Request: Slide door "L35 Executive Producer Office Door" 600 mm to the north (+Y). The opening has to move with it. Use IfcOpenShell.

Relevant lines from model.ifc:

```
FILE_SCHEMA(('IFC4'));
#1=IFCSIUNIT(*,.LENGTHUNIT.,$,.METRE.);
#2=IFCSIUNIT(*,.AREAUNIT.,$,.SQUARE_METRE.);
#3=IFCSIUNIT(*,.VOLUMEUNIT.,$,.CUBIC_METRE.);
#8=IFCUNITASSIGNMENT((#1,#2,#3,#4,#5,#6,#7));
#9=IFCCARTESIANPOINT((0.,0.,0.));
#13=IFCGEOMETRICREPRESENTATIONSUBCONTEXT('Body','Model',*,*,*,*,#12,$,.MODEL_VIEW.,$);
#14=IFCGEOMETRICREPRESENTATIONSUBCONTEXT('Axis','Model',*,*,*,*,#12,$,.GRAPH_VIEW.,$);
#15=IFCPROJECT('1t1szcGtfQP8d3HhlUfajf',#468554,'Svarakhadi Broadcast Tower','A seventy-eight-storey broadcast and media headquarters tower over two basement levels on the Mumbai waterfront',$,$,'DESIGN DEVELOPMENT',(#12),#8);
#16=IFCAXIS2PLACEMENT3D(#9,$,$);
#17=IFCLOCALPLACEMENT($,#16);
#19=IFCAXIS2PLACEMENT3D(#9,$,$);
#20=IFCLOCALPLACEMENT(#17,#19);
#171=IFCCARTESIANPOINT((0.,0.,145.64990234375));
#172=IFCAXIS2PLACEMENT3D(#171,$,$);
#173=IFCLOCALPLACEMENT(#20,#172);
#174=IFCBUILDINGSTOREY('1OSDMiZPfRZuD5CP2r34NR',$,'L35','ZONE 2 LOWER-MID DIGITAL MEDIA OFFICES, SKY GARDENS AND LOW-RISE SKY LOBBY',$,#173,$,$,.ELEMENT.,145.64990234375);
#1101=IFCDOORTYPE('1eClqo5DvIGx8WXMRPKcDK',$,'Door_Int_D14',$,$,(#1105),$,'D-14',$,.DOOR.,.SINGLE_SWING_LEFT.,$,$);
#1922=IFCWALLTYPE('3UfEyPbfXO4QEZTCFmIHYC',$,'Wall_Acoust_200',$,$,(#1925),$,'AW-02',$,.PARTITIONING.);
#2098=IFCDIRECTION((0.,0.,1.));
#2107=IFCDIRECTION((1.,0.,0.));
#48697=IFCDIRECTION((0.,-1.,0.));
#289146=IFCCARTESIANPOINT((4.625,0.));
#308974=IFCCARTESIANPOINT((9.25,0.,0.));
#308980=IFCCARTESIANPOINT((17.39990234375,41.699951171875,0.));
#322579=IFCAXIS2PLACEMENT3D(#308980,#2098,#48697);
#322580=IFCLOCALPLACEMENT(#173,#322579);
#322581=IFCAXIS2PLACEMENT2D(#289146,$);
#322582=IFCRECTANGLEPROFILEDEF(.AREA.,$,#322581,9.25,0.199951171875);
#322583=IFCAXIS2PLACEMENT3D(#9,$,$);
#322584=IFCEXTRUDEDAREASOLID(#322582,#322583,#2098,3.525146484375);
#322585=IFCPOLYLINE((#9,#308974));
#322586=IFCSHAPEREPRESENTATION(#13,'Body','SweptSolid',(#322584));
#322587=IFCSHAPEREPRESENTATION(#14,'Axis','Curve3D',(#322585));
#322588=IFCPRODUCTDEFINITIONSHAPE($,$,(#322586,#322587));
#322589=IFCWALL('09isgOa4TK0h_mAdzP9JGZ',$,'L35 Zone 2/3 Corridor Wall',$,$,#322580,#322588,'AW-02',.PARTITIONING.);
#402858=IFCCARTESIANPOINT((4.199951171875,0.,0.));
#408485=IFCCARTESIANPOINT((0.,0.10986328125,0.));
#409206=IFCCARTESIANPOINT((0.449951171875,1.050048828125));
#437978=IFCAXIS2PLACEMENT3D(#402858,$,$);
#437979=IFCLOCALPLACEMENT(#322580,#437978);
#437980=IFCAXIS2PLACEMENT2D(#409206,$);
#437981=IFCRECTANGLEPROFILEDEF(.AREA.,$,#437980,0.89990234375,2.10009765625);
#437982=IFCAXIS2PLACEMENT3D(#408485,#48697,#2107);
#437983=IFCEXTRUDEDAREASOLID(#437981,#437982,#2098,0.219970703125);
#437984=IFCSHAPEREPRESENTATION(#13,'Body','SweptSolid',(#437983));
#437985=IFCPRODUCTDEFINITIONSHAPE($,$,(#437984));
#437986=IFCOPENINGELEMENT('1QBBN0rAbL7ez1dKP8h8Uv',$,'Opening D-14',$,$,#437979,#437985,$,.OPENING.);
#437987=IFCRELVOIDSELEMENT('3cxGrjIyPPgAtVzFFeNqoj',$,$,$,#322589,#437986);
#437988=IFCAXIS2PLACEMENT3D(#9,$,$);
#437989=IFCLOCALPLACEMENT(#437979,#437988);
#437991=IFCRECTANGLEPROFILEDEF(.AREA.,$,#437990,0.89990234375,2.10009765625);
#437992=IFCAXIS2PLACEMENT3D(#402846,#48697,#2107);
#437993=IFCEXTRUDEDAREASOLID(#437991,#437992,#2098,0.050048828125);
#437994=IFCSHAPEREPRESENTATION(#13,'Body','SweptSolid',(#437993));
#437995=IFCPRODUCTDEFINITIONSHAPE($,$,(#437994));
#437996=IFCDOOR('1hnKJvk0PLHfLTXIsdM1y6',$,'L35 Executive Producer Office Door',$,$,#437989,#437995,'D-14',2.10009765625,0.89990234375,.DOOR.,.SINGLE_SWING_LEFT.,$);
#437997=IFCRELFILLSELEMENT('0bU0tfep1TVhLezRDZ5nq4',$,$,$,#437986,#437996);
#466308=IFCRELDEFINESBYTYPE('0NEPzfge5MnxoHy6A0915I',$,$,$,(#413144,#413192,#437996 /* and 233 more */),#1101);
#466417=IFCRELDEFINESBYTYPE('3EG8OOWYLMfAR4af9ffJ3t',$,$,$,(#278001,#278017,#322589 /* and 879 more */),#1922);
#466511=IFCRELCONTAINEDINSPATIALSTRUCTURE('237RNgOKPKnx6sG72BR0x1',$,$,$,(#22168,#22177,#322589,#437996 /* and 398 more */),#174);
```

```python
import ifcopenshell
import ifcopenshell.api.geometry
import ifcopenshell.util.placement
import ifcopenshell.util.unit

model = ifcopenshell.open("model.ifc")
unit_scale = ifcopenshell.util.unit.calculate_unit_scale(model)

door = model.by_guid("1hnKJvk0PLHfLTXIsdM1y6")
opening = door.FillsVoids[0].RelatingOpeningElement
wall = opening.VoidsElements[0].RelatingBuildingElement

wall_matrix = ifcopenshell.util.placement.get_local_placement(wall.ObjectPlacement)
shift = wall_matrix[:3, 0] * -0.6 / unit_scale
before = ifcopenshell.util.placement.get_local_placement(door.ObjectPlacement)[:3, 3].copy()

# The door is placed relative to its opening, so it follows when the opening moves.
matrix = ifcopenshell.util.placement.get_local_placement(opening.ObjectPlacement)
matrix[:3, 3] += shift
ifcopenshell.api.geometry.edit_object_placement(
    model, product=opening, matrix=matrix, is_si=False, should_transform_children=True
)

after = ifcopenshell.util.placement.get_local_placement(door.ObjectPlacement)[:3, 3]
print("door moved by", (after - before).round(3) + 0.0)

model.write("model_v2.ifc")
```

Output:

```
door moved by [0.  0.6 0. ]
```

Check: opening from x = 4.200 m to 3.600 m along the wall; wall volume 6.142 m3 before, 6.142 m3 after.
